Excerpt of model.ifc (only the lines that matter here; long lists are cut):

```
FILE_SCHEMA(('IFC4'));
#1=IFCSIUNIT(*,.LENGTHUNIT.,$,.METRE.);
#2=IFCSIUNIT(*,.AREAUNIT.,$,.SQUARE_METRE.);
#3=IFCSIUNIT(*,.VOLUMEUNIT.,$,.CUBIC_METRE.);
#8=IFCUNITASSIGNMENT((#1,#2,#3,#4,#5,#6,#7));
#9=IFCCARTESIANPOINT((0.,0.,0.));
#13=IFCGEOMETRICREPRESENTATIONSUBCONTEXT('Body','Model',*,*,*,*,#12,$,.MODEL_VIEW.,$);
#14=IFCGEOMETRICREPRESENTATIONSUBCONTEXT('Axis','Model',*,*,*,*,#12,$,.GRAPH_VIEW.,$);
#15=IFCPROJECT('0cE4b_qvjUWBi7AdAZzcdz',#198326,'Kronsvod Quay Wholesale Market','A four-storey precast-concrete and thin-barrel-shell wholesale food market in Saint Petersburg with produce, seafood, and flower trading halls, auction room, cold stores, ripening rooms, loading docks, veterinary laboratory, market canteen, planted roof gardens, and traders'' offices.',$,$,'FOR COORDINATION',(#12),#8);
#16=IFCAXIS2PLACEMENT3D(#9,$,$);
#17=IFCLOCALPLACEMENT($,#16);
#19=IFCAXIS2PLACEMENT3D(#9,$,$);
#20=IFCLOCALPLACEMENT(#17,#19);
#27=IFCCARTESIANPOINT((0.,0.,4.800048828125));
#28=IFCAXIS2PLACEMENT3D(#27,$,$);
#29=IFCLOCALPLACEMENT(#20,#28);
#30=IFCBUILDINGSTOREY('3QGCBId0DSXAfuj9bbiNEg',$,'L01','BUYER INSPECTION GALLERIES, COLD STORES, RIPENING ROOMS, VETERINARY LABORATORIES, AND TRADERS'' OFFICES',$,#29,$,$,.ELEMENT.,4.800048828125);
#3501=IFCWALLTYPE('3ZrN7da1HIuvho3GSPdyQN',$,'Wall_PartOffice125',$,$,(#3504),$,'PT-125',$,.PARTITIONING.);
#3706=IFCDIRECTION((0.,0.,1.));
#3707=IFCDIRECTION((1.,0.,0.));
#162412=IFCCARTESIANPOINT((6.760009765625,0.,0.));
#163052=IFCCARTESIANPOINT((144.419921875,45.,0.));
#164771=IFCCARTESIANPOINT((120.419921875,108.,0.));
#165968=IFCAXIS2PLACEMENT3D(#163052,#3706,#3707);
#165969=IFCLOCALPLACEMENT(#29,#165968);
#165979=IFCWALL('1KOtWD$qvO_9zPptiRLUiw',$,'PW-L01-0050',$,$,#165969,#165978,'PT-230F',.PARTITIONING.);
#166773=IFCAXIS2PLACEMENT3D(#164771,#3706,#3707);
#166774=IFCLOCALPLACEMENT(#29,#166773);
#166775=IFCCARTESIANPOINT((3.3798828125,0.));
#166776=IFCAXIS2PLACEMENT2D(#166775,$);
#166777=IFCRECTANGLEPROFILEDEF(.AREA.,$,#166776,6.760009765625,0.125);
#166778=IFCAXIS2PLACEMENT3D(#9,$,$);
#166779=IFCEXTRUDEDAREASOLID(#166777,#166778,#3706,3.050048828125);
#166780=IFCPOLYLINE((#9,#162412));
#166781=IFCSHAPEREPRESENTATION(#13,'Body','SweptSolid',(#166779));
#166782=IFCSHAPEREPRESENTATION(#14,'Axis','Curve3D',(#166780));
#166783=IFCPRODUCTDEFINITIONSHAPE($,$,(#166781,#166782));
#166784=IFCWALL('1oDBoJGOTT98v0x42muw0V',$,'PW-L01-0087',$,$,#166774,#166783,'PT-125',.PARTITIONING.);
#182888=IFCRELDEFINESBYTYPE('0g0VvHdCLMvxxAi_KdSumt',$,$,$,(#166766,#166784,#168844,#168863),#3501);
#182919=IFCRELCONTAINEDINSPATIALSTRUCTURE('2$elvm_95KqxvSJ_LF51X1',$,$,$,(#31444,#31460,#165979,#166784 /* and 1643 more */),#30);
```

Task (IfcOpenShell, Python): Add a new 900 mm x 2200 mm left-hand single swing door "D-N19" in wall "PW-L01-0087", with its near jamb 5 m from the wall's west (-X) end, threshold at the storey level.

```python
import numpy as np
import ifcopenshell
import ifcopenshell.api.feature
import ifcopenshell.api.geometry
import ifcopenshell.api.root
import ifcopenshell.api.spatial
import ifcopenshell.geom
import ifcopenshell.util.element
import ifcopenshell.util.placement
import ifcopenshell.util.representation
import ifcopenshell.util.shape
import ifcopenshell.util.unit

model = ifcopenshell.open("model.ifc")
unit_scale = ifcopenshell.util.unit.calculate_unit_scale(model)
settings = ifcopenshell.geom.settings()


def volume(element):
    """Net volume in cubic metres, openings subtracted."""
    shape = ifcopenshell.geom.create_shape(settings, element)
    return ifcopenshell.util.shape.get_volume(shape.geometry)


wall = model.by_id(166784)
storey = ifcopenshell.util.element.get_container(wall, ifc_class="IfcBuildingStorey")
context = ifcopenshell.util.representation.get_context(model, "Model", "Body", "MODEL_VIEW")
before = volume(wall)

width, height, from_end, sill = 0.9, 2.2, 5, 0.0  # metres

# The wall runs along its own X axis, and the end named is its -X end.
wall_shape = ifcopenshell.geom.create_shape(settings, wall)
x, y, z = ifcopenshell.util.shape.get_vertices(wall_shape.geometry).T
start = x.min() + from_end
face, thickness = float(y.min()), float(y.max() - y.min())
wall_matrix = ifcopenshell.util.placement.get_local_placement(wall.ObjectPlacement)
level = ifcopenshell.util.placement.get_local_placement(storey.ObjectPlacement)[2, 3]


def in_wall(x, y):
    """Placement at x, y metres in the wall's axes, at sill height."""
    matrix = wall_matrix.copy()
    matrix[:, 3] = wall_matrix @ np.array([x / unit_scale, y / unit_scale, 0.0, 1.0])
    matrix[2, 3] = level + sill / unit_scale
    return matrix


# Opening: a box that overshoots both wall faces by 50 mm.
opening = ifcopenshell.api.root.create_entity(model, ifc_class="IfcOpeningElement", predefined_type="OPENING")
box = ifcopenshell.api.geometry.add_wall_representation(
    model, context=context, length=width, height=height, thickness=thickness + 0.1
)
ifcopenshell.api.geometry.assign_representation(model, product=opening, representation=box)
ifcopenshell.api.geometry.edit_object_placement(model, product=opening, matrix=in_wall(start, face - 0.05), is_si=False)
ifcopenshell.api.feature.add_feature(model, feature=opening, element=wall)

door = ifcopenshell.api.root.create_entity(model, ifc_class="IfcDoor", name="D-N19", predefined_type="DOOR")
door.OverallWidth, door.OverallHeight = width / unit_scale, height / unit_scale
door.OperationType = "SINGLE_SWING_LEFT"
body = ifcopenshell.api.geometry.add_door_representation(
    model,
    context=context,
    overall_width=door.OverallWidth,
    overall_height=door.OverallHeight,
    operation_type="SINGLE_SWING_LEFT",
    lining_properties={"LiningDepth": thickness / unit_scale, "ThresholdDepth": thickness / unit_scale},
)
ifcopenshell.api.geometry.assign_representation(model, product=door, representation=body)
ifcopenshell.api.spatial.assign_container(model, products=[door], relating_structure=storey)
ifcopenshell.api.feature.add_filling(model, opening=opening, element=door)

# The lining spans the wall, so the door starts at the wall face.
ifcopenshell.api.geometry.edit_object_placement(model, product=door, matrix=in_wall(start, face), is_si=False)

after = volume(wall)

print(f"wall volume {before:.3f} -> {after:.3f} m3")

model.write("model-out.ifc")
```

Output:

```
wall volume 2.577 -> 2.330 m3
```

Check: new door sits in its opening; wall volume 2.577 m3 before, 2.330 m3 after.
